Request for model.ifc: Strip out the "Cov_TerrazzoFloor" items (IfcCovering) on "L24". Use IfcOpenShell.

First a look at what the model holds.

```python
import ifcopenshell
import ifcopenshell.util.element

model = ifcopenshell.open("model.ifc")
print(model.schema)
storey = next(s for s in model.by_type("IfcBuildingStorey") if s.Name == "L24")
coverings = [e for e in ifcopenshell.util.element.get_decomposition(storey) if e.is_a("IfcCovering")]
seen = {}
for e in coverings:
    element_type = ifcopenshell.util.element.get_type(e)
    name = element_type.Name if element_type not in (None, e) else None
    seen[name] = seen.get(name, 0) + 1
for name, count in sorted(seen.items(), key=str):
    print(count, "x", name)
```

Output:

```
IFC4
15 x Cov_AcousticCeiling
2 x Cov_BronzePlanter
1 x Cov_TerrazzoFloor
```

```python
import ifcopenshell
import ifcopenshell.api.root
import ifcopenshell.util.element

model = ifcopenshell.open("model.ifc")

storey = next(s for s in model.by_type("IfcBuildingStorey") if s.Name == "L24")
coverings = [e for e in ifcopenshell.util.element.get_decomposition(storey) if e.is_a("IfcCovering")]
targets = [e for e in coverings if (t := ifcopenshell.util.element.get_type(e)) not in (None, e) and t.Name == "Cov_TerrazzoFloor"]

for e in targets:
    ifcopenshell.api.root.remove_product(model, product=e)
print(len(targets), "removed")

model.write("model-out.ifc")
```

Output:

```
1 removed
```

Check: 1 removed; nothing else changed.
